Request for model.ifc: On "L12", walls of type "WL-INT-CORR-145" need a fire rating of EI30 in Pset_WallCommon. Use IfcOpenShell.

First a look at what the model holds.

```python
import ifcopenshell
import ifcopenshell.util.element

model = ifcopenshell.open("model.ifc")
print(model.schema)
storey = next(s for s in model.by_type("IfcBuildingStorey") if s.Name == "L12")
walls = [e for e in ifcopenshell.util.element.get_decomposition(storey) if e.is_a("IfcWall")]
seen = {}
for e in walls:
    element_type = ifcopenshell.util.element.get_type(e)
    key = (element_type.Name if element_type != e and element_type else None, ifcopenshell.util.element.get_pset(e, "Pset_WallCommon", "FireRating"))
    seen[key] = seen.get(key, 0) + 1
for (name, value), count in sorted(seen.items(), key=str):
    print(count, "x", name, "|", value)
```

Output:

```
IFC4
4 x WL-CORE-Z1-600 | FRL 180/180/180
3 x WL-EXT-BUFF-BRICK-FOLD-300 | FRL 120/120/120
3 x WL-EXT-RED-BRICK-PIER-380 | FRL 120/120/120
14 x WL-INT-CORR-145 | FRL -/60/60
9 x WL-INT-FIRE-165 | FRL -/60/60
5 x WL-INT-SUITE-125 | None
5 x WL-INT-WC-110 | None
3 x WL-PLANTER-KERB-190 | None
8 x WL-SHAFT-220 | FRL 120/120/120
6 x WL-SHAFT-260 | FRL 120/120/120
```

```python
import ifcopenshell
import ifcopenshell.api.pset
import ifcopenshell.util.element

model = ifcopenshell.open("model.ifc")

storey = next(s for s in model.by_type("IfcBuildingStorey") if s.Name == "L12")
walls = [e for e in ifcopenshell.util.element.get_decomposition(storey) if e.is_a("IfcWall")]

count = 0
for e in walls:
    element_type = ifcopenshell.util.element.get_type(e)
    if element_type in (None, e) or element_type.Name != "WL-INT-CORR-145":
        continue
    found = ifcopenshell.util.element.get_pset(e, "Pset_WallCommon", should_inherit=False)
    if found:
        pset = model.by_id(found["id"])
        if len(ifcopenshell.util.element.get_elements_by_pset(pset)) > 1:
            pset = ifcopenshell.api.pset.unshare_pset(model, products=[e], pset=pset)[0]
    else:
        pset = ifcopenshell.api.pset.add_pset(model, product=e, name="Pset_WallCommon")
    ifcopenshell.api.pset.edit_pset(model, pset=pset, properties={"FireRating": "EI30"})
    count += 1

print(count, "walls updated")

model.write("model-out.ifc")
```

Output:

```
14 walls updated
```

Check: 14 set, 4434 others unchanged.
